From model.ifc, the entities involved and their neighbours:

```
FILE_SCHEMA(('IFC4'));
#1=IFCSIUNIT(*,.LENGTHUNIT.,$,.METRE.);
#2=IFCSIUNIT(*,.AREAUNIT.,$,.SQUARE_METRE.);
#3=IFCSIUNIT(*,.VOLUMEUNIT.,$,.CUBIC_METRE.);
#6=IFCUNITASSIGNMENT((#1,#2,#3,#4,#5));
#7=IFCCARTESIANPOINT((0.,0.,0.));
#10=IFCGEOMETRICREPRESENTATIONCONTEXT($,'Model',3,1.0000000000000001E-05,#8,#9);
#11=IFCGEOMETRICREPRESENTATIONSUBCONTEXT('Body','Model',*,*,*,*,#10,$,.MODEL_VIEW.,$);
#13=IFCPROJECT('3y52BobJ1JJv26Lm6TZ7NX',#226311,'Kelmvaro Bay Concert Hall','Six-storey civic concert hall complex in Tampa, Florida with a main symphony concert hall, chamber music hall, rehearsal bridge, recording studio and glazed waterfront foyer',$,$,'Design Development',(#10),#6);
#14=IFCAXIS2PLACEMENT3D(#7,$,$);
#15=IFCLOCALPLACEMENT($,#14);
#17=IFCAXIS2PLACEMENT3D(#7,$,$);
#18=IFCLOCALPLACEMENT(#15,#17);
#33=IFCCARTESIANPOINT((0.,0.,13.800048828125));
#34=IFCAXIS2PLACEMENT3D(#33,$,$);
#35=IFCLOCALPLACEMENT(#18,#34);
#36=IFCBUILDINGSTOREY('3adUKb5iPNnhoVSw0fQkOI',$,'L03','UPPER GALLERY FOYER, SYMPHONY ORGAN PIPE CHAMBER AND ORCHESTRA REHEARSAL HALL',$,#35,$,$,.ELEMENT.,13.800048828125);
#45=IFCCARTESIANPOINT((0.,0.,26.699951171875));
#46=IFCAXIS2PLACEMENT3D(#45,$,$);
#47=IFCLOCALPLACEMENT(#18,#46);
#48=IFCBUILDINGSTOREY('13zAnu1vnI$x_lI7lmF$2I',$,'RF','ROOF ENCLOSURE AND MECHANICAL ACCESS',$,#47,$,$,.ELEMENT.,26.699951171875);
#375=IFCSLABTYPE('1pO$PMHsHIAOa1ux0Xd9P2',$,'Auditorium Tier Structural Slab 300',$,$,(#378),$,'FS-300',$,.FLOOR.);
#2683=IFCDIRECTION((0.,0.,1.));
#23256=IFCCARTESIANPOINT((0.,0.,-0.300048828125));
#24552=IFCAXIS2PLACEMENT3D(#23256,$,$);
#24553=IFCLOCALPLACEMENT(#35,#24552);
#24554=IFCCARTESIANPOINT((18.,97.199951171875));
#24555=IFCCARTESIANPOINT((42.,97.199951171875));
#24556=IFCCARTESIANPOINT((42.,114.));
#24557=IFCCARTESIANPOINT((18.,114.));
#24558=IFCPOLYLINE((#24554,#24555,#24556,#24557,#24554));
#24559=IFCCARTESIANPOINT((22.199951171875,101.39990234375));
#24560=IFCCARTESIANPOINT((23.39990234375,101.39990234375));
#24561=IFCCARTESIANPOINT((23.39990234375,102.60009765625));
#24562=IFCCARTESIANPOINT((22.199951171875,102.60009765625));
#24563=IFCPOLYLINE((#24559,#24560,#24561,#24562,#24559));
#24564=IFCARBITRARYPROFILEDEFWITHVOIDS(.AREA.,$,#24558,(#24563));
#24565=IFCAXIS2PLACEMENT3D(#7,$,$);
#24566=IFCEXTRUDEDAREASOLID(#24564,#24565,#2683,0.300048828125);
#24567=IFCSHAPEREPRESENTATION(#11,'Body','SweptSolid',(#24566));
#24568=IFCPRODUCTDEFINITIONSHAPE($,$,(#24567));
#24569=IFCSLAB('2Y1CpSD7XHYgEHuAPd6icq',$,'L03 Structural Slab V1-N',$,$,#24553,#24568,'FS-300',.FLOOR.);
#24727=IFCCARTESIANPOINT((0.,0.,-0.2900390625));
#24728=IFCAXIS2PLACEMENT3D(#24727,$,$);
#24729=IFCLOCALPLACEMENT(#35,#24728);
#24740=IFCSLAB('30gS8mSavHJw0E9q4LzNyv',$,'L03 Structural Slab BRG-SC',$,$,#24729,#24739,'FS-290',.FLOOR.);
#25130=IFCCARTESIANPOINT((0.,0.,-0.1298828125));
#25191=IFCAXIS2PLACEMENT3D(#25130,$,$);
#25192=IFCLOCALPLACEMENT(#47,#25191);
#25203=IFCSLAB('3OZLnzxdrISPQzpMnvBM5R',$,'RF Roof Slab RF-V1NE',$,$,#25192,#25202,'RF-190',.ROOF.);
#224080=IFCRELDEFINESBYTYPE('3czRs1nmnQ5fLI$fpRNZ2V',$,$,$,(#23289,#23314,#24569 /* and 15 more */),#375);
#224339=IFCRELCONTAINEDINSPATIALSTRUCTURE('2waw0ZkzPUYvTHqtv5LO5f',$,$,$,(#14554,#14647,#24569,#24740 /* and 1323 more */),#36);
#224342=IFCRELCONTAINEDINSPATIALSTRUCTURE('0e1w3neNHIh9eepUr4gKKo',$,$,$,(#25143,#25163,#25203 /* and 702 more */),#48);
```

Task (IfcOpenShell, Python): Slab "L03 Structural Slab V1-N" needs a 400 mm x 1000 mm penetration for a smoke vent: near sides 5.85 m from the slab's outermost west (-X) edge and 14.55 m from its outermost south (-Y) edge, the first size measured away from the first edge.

```python
import numpy as np
import ifcopenshell
import ifcopenshell.api.feature
import ifcopenshell.api.geometry
import ifcopenshell.api.root
import ifcopenshell.geom
import ifcopenshell.util.placement
import ifcopenshell.util.representation
import ifcopenshell.util.shape
import ifcopenshell.util.unit

model = ifcopenshell.open("model.ifc")
unit_scale = ifcopenshell.util.unit.calculate_unit_scale(model)
settings = ifcopenshell.geom.settings()


def volume(element):
    """Net volume in cubic metres, openings subtracted."""
    shape = ifcopenshell.geom.create_shape(settings, element)
    return ifcopenshell.util.shape.get_volume(shape.geometry)


slab = model.by_guid("2Y1CpSD7XHYgEHuAPd6icq")
before = volume(slab)

# Extent in the slab's own axes, in metres. The edges named are its -X and -Y sides.
slab_shape = ifcopenshell.geom.create_shape(settings, slab)
vertices = ifcopenshell.util.shape.get_vertices(slab_shape.geometry)
x_min, y_min, bottom = vertices.min(axis=0)
top = vertices[:, 2].max()

opening = ifcopenshell.api.root.create_entity(model, ifc_class="IfcOpeningElement", name="Smoke vent opening", predefined_type="OPENING")
context = ifcopenshell.util.representation.get_context(model, "Model", "Body", "MODEL_VIEW")
width, depth = 0.4, 1
outline = [(0.0, 0.0), (width, 0.0), (width, depth), (0.0, depth), (0.0, 0.0)]
# Overshoot both faces by 50 mm so the cut is clean.
shape = ifcopenshell.api.geometry.add_slab_representation(
    model, context=context, depth=top - bottom + 0.1, polyline=outline
)
ifcopenshell.api.geometry.assign_representation(model, product=opening, representation=shape)

matrix = ifcopenshell.util.placement.get_local_placement(slab.ObjectPlacement)
matrix[:, 3] = matrix @ np.append(np.array([x_min + 5.85, y_min + 14.55, bottom - 0.05]) / unit_scale, 1.0)
ifcopenshell.api.geometry.edit_object_placement(model, product=opening, matrix=matrix, is_si=False)
ifcopenshell.api.feature.add_feature(model, feature=opening, element=slab)

after = volume(slab)

print(f"slab volume {before:.3f} -> {after:.3f} m3")

model.write("model_rev.ifc")
```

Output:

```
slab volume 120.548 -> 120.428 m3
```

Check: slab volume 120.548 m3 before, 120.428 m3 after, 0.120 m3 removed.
